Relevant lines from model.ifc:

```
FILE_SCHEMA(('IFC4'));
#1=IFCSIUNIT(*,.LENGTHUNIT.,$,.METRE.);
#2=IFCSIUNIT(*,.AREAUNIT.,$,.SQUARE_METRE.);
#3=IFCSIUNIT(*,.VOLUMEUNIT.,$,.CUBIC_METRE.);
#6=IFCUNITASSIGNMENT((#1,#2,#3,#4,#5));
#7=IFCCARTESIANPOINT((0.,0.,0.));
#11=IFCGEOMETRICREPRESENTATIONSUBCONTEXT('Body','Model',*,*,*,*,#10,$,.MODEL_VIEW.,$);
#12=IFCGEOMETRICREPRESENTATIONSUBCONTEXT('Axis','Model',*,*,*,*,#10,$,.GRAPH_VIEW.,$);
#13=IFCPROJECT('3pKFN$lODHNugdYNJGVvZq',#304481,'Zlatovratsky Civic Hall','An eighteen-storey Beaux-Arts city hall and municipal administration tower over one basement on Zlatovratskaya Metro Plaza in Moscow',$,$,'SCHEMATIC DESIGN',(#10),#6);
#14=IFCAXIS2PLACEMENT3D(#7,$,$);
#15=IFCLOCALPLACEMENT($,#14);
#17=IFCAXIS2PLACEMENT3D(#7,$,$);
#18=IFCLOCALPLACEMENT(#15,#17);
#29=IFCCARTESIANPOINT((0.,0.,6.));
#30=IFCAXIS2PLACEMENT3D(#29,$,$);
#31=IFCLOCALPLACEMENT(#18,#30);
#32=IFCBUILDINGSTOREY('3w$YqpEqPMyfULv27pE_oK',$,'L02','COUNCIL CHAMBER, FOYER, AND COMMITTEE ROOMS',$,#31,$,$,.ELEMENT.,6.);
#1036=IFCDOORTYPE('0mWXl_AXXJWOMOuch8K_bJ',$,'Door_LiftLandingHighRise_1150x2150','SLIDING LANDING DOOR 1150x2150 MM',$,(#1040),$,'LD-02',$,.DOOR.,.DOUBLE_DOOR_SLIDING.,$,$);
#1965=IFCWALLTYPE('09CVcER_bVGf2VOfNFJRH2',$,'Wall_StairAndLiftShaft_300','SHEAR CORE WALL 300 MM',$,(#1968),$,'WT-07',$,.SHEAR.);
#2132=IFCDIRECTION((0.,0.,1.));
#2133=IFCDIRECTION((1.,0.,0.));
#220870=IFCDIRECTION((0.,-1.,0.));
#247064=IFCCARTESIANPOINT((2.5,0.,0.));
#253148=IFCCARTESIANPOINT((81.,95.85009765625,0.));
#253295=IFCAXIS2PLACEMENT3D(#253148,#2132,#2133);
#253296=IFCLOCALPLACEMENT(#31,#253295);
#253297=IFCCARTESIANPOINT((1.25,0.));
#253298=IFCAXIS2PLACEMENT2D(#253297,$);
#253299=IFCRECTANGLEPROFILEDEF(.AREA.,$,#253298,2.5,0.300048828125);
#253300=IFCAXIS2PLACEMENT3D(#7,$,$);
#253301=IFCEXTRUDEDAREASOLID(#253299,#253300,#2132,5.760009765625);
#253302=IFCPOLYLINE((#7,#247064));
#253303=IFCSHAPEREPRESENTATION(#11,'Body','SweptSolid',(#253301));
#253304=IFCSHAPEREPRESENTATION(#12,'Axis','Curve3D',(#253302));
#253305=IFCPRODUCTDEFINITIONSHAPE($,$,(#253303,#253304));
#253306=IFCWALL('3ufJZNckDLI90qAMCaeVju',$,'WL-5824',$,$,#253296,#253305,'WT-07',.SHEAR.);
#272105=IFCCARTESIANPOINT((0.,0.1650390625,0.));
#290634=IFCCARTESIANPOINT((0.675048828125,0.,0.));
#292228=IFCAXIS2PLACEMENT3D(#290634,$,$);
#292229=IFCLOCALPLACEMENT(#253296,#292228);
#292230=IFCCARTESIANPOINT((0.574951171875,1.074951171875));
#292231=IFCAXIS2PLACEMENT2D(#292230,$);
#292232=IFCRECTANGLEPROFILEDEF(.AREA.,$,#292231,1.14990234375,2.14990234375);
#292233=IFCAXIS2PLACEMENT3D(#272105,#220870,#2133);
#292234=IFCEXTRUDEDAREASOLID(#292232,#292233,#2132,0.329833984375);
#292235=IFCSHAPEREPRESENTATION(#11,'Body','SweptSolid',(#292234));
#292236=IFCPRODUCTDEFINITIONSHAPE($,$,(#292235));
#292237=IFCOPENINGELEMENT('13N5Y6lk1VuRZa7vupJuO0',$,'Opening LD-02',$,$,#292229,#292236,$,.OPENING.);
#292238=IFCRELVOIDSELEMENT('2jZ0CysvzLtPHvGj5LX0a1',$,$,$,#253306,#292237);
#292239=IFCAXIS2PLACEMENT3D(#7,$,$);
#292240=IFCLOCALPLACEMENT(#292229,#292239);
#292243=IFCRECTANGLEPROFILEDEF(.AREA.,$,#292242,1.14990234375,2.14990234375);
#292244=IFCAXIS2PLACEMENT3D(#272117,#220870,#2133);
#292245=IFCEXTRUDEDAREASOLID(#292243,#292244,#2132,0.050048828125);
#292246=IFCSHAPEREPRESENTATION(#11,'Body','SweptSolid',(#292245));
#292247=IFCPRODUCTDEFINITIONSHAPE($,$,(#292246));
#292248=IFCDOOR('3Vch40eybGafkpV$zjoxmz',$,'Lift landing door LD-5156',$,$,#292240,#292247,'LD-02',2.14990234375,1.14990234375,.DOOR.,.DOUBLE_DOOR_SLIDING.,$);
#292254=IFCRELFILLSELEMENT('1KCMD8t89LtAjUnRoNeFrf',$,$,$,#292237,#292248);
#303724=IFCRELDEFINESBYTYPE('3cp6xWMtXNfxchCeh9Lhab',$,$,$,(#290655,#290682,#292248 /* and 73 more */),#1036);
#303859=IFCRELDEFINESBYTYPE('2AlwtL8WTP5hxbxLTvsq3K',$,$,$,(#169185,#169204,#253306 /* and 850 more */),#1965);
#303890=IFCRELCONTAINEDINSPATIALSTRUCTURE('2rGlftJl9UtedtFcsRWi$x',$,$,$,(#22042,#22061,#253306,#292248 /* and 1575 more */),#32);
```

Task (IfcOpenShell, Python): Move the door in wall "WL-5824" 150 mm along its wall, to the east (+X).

```python
import ifcopenshell
import ifcopenshell.api.geometry
import ifcopenshell.util.placement

model = ifcopenshell.open("model.ifc")

door = model.by_id(292248)
opening = door.FillsVoids[0].RelatingOpeningElement
wall = opening.VoidsElements[0].RelatingBuildingElement

wall_matrix = ifcopenshell.util.placement.get_local_placement(wall.ObjectPlacement)
shift = wall_matrix[:3, 0] * 0.15
before = ifcopenshell.util.placement.get_local_placement(door.ObjectPlacement)[:3, 3].copy()

# The door is placed relative to its opening, so it follows when the opening moves.
matrix = ifcopenshell.util.placement.get_local_placement(opening.ObjectPlacement)
matrix[:3, 3] += shift
ifcopenshell.api.geometry.edit_object_placement(
    model, product=opening, matrix=matrix, is_si=False, should_transform_children=True
)

after = ifcopenshell.util.placement.get_local_placement(door.ObjectPlacement)[:3, 3]
print("door moved by", (after - before).round(3) + 0.0)

model.write("model_edited.ifc")
```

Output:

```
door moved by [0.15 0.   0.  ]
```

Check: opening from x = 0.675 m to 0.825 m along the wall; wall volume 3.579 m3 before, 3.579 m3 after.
